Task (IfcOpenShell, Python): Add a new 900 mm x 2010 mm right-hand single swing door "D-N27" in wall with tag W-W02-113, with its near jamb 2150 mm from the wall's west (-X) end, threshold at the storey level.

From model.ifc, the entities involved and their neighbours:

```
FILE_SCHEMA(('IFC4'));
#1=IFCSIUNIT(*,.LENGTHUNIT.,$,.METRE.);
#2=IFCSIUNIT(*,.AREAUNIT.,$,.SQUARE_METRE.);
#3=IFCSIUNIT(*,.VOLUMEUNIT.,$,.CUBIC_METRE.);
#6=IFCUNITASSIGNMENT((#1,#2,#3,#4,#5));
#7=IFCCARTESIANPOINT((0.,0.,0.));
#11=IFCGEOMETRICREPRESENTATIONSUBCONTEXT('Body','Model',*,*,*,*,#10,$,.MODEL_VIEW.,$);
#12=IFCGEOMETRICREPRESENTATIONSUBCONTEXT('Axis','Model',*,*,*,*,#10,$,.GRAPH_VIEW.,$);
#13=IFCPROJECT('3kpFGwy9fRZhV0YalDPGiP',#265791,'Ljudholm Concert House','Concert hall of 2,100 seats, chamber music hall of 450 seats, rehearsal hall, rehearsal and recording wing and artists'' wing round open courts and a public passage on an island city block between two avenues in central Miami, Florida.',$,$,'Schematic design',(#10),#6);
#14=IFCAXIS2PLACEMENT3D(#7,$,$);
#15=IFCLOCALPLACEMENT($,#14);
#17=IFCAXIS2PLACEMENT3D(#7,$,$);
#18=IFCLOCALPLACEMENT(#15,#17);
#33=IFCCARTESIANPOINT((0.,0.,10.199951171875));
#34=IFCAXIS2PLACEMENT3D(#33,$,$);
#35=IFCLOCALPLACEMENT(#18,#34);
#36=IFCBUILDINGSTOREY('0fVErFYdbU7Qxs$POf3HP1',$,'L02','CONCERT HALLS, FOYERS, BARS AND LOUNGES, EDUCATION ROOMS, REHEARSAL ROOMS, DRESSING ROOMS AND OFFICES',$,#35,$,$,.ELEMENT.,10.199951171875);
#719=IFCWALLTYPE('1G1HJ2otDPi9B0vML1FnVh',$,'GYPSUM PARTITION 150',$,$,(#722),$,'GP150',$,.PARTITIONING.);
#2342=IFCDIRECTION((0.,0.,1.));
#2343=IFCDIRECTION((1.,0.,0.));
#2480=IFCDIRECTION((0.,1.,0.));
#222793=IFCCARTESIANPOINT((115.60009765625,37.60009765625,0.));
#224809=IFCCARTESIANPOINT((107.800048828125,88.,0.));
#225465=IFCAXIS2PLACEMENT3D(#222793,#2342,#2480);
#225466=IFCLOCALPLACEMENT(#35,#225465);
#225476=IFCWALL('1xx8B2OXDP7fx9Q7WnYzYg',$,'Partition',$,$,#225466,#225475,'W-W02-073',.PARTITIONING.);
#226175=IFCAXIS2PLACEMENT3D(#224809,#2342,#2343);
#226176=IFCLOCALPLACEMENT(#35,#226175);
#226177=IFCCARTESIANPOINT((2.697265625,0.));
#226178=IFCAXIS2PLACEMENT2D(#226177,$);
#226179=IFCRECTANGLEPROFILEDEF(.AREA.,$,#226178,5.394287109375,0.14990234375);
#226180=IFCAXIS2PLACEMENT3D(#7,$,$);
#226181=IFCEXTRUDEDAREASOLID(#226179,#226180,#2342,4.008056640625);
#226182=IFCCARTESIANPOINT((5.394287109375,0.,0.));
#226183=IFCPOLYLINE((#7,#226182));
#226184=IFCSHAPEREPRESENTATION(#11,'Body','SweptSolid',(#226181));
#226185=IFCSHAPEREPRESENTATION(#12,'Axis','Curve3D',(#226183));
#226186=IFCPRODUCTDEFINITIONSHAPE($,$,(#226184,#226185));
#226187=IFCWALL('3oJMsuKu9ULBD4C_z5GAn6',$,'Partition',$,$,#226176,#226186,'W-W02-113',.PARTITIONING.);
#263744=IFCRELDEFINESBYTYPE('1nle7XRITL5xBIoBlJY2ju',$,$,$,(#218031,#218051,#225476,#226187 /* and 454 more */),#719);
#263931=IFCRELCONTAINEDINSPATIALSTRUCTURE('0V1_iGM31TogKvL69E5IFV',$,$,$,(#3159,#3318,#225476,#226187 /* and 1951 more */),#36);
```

```python
import numpy as np
import ifcopenshell
import ifcopenshell.api.feature
import ifcopenshell.api.geometry
import ifcopenshell.api.root
import ifcopenshell.api.spatial
import ifcopenshell.geom
import ifcopenshell.util.element
import ifcopenshell.util.placement
import ifcopenshell.util.representation
import ifcopenshell.util.shape
import ifcopenshell.util.unit

model = ifcopenshell.open("model.ifc")
unit_scale = ifcopenshell.util.unit.calculate_unit_scale(model)
settings = ifcopenshell.geom.settings()


def volume(element):
    """Net volume in cubic metres, openings subtracted."""
    shape = ifcopenshell.geom.create_shape(settings, element)
    return ifcopenshell.util.shape.get_volume(shape.geometry)


wall = model.by_guid("3oJMsuKu9ULBD4C_z5GAn6")
storey = ifcopenshell.util.element.get_container(wall, ifc_class="IfcBuildingStorey")
context = ifcopenshell.util.representation.get_context(model, "Model", "Body", "MODEL_VIEW")
before = volume(wall)

width, height, from_end, sill = 0.9, 2.01, 2.15, 0.0  # metres

# The wall runs along its own X axis, and the end named is its -X end.
wall_shape = ifcopenshell.geom.create_shape(settings, wall)
x, y, z = ifcopenshell.util.shape.get_vertices(wall_shape.geometry).T
start = x.min() + from_end
face, thickness = float(y.min()), float(y.max() - y.min())
wall_matrix = ifcopenshell.util.placement.get_local_placement(wall.ObjectPlacement)
level = ifcopenshell.util.placement.get_local_placement(storey.ObjectPlacement)[2, 3]


def in_wall(x, y):
    """Placement at x, y metres in the wall's axes, at sill height."""
    matrix = wall_matrix.copy()
    matrix[:, 3] = wall_matrix @ np.array([x / unit_scale, y / unit_scale, 0.0, 1.0])
    matrix[2, 3] = level + sill / unit_scale
    return matrix


# Opening: a box that overshoots both wall faces by 50 mm.
opening = ifcopenshell.api.root.create_entity(model, ifc_class="IfcOpeningElement", predefined_type="OPENING")
box = ifcopenshell.api.geometry.add_wall_representation(
    model, context=context, length=width, height=height, thickness=thickness + 0.1
)
ifcopenshell.api.geometry.assign_representation(model, product=opening, representation=box)
ifcopenshell.api.geometry.edit_object_placement(model, product=opening, matrix=in_wall(start, face - 0.05), is_si=False)
ifcopenshell.api.feature.add_feature(model, feature=opening, element=wall)

door = ifcopenshell.api.root.create_entity(model, ifc_class="IfcDoor", name="D-N27", predefined_type="DOOR")
door.OverallWidth, door.OverallHeight = width / unit_scale, height / unit_scale
door.OperationType = "SINGLE_SWING_RIGHT"
body = ifcopenshell.api.geometry.add_door_representation(
    model,
    context=context,
    overall_width=door.OverallWidth,
    overall_height=door.OverallHeight,
    operation_type="SINGLE_SWING_RIGHT",
    lining_properties={"LiningDepth": thickness / unit_scale, "ThresholdDepth": thickness / unit_scale},
)
ifcopenshell.api.geometry.assign_representation(model, product=door, representation=body)
ifcopenshell.api.spatial.assign_container(model, products=[door], relating_structure=storey)
ifcopenshell.api.feature.add_filling(model, opening=opening, element=door)

# The lining spans the wall, so the door starts at the wall face.
ifcopenshell.api.geometry.edit_object_placement(model, product=door, matrix=in_wall(start, face), is_si=False)

after = volume(wall)

print(f"wall volume {before:.3f} -> {after:.3f} m3")

model.write("model-out.ifc")
```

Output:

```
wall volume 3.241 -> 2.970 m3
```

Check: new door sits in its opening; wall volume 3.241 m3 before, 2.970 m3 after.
